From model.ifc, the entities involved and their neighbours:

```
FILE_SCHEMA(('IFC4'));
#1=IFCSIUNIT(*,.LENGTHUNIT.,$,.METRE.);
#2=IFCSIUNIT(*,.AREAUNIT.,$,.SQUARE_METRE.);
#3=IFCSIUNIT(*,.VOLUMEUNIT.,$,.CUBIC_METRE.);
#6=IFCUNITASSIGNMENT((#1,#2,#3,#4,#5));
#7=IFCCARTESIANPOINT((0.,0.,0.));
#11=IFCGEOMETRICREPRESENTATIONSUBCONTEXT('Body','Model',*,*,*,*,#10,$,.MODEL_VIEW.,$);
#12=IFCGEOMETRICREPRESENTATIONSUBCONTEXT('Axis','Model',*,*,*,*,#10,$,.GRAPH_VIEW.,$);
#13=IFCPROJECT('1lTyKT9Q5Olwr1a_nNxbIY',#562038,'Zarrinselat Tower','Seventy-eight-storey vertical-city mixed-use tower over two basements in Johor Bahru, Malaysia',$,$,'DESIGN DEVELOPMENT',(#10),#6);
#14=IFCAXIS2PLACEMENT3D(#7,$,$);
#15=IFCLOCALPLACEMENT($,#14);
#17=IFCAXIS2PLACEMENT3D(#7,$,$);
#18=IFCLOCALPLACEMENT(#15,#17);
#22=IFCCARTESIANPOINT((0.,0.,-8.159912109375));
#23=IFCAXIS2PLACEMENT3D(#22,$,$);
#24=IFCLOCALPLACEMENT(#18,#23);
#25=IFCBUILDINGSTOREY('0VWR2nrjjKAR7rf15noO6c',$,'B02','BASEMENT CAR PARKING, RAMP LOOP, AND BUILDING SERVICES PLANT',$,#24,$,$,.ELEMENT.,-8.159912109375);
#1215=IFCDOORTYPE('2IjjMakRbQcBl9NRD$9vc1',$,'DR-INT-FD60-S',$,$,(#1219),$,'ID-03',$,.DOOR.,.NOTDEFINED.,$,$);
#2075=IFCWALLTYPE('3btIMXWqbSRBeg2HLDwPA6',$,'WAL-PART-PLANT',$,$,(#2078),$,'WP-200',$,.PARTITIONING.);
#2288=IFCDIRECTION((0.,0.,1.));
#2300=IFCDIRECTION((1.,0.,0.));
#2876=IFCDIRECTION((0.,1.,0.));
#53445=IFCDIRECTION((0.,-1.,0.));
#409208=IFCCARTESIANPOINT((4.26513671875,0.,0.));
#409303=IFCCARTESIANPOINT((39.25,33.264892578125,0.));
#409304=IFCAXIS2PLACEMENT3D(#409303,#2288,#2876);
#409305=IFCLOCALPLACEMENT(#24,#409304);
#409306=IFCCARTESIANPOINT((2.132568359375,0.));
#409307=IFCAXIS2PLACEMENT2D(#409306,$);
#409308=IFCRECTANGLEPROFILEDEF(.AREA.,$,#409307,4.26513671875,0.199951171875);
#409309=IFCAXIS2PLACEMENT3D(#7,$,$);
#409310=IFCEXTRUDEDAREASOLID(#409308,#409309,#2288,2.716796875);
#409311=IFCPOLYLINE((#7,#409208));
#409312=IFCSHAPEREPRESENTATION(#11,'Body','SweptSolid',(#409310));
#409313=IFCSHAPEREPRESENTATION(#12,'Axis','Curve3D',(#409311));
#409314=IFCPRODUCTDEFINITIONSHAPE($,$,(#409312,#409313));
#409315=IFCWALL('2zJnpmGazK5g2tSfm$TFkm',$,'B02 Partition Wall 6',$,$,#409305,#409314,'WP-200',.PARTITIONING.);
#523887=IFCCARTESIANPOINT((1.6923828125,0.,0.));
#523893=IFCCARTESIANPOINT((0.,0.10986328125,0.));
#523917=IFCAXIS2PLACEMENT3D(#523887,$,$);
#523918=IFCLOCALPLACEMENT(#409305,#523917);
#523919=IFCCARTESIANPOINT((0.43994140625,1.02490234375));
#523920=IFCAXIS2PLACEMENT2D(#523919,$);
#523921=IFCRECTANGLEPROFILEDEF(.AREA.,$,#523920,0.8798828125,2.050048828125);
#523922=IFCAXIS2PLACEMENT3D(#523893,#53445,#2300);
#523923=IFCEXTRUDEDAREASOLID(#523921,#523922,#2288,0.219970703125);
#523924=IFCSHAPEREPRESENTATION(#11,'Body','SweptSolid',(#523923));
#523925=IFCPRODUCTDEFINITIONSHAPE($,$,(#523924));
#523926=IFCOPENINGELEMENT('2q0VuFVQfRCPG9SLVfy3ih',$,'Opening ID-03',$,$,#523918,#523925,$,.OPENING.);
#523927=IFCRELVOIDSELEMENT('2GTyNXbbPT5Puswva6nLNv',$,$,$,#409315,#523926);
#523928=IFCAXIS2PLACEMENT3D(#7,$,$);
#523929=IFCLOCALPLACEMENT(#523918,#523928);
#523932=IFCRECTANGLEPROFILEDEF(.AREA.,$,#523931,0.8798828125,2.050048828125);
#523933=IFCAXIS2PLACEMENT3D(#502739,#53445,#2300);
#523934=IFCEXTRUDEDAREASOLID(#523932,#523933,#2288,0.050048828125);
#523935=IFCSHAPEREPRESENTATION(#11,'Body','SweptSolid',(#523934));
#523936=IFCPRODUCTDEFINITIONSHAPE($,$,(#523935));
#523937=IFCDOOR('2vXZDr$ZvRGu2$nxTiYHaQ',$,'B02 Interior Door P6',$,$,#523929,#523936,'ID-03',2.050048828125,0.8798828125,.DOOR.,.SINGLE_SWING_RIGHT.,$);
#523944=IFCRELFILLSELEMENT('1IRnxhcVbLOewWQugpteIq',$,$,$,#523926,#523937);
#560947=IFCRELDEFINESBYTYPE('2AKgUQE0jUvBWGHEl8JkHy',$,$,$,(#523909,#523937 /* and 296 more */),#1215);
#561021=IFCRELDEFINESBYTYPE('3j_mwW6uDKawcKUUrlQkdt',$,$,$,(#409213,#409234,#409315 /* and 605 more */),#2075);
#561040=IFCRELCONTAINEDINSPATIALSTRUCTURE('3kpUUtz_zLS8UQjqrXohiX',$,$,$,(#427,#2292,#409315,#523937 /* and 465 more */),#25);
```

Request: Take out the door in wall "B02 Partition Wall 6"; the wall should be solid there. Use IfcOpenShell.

```python
import ifcopenshell
import ifcopenshell.api.feature
import ifcopenshell.api.root
import ifcopenshell.geom
import ifcopenshell.util.shape

model = ifcopenshell.open("model.ifc")
settings = ifcopenshell.geom.settings()


def volume(element):
    """Net volume in cubic metres, openings subtracted."""
    shape = ifcopenshell.geom.create_shape(settings, element)
    return ifcopenshell.util.shape.get_volume(shape.geometry)


door = model.by_id(523937)
opening = door.FillsVoids[0].RelatingOpeningElement
wall = opening.VoidsElements[0].RelatingBuildingElement
before = volume(wall)

ifcopenshell.api.root.remove_product(model, product=door)
ifcopenshell.api.feature.remove_feature(model, feature=opening)

after = volume(wall)

print(f"wall volume {before:.3f} -> {after:.3f} m3")

model.write("model_updated.ifc")
```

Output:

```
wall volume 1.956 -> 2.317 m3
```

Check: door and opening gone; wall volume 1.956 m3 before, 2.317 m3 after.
